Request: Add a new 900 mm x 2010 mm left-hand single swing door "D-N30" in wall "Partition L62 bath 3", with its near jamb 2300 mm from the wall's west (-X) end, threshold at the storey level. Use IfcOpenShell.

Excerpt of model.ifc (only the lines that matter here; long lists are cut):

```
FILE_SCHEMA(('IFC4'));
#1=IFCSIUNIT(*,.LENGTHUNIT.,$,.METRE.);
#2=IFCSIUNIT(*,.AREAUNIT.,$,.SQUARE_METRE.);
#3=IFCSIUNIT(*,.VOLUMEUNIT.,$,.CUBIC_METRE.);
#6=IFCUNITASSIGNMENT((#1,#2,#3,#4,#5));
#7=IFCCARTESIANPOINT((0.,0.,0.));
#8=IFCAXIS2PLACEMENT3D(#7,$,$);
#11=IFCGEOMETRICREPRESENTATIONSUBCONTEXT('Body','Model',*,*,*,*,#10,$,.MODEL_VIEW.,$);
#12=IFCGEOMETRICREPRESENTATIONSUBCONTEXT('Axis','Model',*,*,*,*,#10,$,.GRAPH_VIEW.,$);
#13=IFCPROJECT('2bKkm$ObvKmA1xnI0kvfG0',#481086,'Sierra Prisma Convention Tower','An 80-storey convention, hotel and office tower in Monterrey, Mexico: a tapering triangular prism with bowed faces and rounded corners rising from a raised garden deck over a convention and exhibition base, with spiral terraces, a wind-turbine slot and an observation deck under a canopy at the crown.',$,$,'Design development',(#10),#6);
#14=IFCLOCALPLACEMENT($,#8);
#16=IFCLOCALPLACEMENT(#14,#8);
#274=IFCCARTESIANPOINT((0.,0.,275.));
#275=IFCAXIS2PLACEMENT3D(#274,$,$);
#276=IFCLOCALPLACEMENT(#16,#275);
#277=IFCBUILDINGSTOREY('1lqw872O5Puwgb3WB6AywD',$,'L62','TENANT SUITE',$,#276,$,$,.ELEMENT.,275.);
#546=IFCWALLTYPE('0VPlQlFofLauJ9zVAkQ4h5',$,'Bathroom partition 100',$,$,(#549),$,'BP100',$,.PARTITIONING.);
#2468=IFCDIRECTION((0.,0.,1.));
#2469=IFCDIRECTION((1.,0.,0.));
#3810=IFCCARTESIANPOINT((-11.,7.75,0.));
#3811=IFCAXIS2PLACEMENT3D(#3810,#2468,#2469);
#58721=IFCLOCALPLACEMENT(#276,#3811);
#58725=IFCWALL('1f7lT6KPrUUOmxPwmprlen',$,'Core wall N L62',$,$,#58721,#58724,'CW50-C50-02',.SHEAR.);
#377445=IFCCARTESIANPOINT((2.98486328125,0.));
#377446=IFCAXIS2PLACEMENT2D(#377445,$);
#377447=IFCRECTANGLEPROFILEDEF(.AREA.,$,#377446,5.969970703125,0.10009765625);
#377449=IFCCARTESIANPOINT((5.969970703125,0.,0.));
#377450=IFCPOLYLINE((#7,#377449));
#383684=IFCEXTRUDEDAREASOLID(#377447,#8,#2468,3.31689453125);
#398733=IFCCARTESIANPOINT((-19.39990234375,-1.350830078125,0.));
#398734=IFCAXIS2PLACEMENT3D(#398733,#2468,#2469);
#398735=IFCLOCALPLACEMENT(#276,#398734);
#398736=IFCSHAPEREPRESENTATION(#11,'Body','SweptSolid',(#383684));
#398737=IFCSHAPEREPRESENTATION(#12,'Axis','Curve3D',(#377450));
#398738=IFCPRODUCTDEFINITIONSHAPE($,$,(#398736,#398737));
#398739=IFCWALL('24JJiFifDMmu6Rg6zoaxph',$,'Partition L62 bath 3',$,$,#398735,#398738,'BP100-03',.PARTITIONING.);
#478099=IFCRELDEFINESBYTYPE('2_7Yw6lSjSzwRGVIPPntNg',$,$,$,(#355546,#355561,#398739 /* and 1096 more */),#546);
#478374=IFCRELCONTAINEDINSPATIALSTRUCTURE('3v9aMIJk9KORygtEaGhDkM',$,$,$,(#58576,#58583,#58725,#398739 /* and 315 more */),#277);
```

```python
import numpy as np
import ifcopenshell
import ifcopenshell.api.feature
import ifcopenshell.api.geometry
import ifcopenshell.api.root
import ifcopenshell.api.spatial
import ifcopenshell.geom
import ifcopenshell.util.element
import ifcopenshell.util.placement
import ifcopenshell.util.representation
import ifcopenshell.util.shape
import ifcopenshell.util.unit

model = ifcopenshell.open("model.ifc")
unit_scale = ifcopenshell.util.unit.calculate_unit_scale(model)
settings = ifcopenshell.geom.settings()


def volume(element):
    """Net volume in cubic metres, openings subtracted."""
    shape = ifcopenshell.geom.create_shape(settings, element)
    return ifcopenshell.util.shape.get_volume(shape.geometry)


wall = model.by_guid("24JJiFifDMmu6Rg6zoaxph")
storey = ifcopenshell.util.element.get_container(wall, ifc_class="IfcBuildingStorey")
context = ifcopenshell.util.representation.get_context(model, "Model", "Body", "MODEL_VIEW")
before = volume(wall)

width, height, from_end, sill = 0.9, 2.01, 2.3, 0.0  # metres

# The wall runs along its own X axis, and the end named is its -X end.
wall_shape = ifcopenshell.geom.create_shape(settings, wall)
x, y, z = ifcopenshell.util.shape.get_vertices(wall_shape.geometry).T
start = x.min() + from_end
face, thickness = float(y.min()), float(y.max() - y.min())
wall_matrix = ifcopenshell.util.placement.get_local_placement(wall.ObjectPlacement)
level = ifcopenshell.util.placement.get_local_placement(storey.ObjectPlacement)[2, 3]


def in_wall(x, y):
    """Placement at x, y metres in the wall's axes, at sill height."""
    matrix = wall_matrix.copy()
    matrix[:, 3] = wall_matrix @ np.array([x / unit_scale, y / unit_scale, 0.0, 1.0])
    matrix[2, 3] = level + sill / unit_scale
    return matrix


# Opening: a box that overshoots both wall faces by 50 mm.
opening = ifcopenshell.api.root.create_entity(model, ifc_class="IfcOpeningElement", predefined_type="OPENING")
box = ifcopenshell.api.geometry.add_wall_representation(
    model, context=context, length=width, height=height, thickness=thickness + 0.1
)
ifcopenshell.api.geometry.assign_representation(model, product=opening, representation=box)
ifcopenshell.api.geometry.edit_object_placement(model, product=opening, matrix=in_wall(start, face - 0.05), is_si=False)
ifcopenshell.api.feature.add_feature(model, feature=opening, element=wall)

door = ifcopenshell.api.root.create_entity(model, ifc_class="IfcDoor", name="D-N30", predefined_type="DOOR")
door.OverallWidth, door.OverallHeight = width / unit_scale, height / unit_scale
door.OperationType = "SINGLE_SWING_LEFT"
body = ifcopenshell.api.geometry.add_door_representation(
    model,
    context=context,
    overall_width=door.OverallWidth,
    overall_height=door.OverallHeight,
    operation_type="SINGLE_SWING_LEFT",
    lining_properties={"LiningDepth": thickness / unit_scale, "ThresholdDepth": thickness / unit_scale},
)
ifcopenshell.api.geometry.assign_representation(model, product=door, representation=body)
ifcopenshell.api.spatial.assign_container(model, products=[door], relating_structure=storey)
ifcopenshell.api.feature.add_filling(model, opening=opening, element=door)

# The lining spans the wall, so the door starts at the wall face.
ifcopenshell.api.geometry.edit_object_placement(model, product=door, matrix=in_wall(start, face), is_si=False)

after = volume(wall)

print(f"wall volume {before:.3f} -> {after:.3f} m3")

model.write("model_rev.ifc")
```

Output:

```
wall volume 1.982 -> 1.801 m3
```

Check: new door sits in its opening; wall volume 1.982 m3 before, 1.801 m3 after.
